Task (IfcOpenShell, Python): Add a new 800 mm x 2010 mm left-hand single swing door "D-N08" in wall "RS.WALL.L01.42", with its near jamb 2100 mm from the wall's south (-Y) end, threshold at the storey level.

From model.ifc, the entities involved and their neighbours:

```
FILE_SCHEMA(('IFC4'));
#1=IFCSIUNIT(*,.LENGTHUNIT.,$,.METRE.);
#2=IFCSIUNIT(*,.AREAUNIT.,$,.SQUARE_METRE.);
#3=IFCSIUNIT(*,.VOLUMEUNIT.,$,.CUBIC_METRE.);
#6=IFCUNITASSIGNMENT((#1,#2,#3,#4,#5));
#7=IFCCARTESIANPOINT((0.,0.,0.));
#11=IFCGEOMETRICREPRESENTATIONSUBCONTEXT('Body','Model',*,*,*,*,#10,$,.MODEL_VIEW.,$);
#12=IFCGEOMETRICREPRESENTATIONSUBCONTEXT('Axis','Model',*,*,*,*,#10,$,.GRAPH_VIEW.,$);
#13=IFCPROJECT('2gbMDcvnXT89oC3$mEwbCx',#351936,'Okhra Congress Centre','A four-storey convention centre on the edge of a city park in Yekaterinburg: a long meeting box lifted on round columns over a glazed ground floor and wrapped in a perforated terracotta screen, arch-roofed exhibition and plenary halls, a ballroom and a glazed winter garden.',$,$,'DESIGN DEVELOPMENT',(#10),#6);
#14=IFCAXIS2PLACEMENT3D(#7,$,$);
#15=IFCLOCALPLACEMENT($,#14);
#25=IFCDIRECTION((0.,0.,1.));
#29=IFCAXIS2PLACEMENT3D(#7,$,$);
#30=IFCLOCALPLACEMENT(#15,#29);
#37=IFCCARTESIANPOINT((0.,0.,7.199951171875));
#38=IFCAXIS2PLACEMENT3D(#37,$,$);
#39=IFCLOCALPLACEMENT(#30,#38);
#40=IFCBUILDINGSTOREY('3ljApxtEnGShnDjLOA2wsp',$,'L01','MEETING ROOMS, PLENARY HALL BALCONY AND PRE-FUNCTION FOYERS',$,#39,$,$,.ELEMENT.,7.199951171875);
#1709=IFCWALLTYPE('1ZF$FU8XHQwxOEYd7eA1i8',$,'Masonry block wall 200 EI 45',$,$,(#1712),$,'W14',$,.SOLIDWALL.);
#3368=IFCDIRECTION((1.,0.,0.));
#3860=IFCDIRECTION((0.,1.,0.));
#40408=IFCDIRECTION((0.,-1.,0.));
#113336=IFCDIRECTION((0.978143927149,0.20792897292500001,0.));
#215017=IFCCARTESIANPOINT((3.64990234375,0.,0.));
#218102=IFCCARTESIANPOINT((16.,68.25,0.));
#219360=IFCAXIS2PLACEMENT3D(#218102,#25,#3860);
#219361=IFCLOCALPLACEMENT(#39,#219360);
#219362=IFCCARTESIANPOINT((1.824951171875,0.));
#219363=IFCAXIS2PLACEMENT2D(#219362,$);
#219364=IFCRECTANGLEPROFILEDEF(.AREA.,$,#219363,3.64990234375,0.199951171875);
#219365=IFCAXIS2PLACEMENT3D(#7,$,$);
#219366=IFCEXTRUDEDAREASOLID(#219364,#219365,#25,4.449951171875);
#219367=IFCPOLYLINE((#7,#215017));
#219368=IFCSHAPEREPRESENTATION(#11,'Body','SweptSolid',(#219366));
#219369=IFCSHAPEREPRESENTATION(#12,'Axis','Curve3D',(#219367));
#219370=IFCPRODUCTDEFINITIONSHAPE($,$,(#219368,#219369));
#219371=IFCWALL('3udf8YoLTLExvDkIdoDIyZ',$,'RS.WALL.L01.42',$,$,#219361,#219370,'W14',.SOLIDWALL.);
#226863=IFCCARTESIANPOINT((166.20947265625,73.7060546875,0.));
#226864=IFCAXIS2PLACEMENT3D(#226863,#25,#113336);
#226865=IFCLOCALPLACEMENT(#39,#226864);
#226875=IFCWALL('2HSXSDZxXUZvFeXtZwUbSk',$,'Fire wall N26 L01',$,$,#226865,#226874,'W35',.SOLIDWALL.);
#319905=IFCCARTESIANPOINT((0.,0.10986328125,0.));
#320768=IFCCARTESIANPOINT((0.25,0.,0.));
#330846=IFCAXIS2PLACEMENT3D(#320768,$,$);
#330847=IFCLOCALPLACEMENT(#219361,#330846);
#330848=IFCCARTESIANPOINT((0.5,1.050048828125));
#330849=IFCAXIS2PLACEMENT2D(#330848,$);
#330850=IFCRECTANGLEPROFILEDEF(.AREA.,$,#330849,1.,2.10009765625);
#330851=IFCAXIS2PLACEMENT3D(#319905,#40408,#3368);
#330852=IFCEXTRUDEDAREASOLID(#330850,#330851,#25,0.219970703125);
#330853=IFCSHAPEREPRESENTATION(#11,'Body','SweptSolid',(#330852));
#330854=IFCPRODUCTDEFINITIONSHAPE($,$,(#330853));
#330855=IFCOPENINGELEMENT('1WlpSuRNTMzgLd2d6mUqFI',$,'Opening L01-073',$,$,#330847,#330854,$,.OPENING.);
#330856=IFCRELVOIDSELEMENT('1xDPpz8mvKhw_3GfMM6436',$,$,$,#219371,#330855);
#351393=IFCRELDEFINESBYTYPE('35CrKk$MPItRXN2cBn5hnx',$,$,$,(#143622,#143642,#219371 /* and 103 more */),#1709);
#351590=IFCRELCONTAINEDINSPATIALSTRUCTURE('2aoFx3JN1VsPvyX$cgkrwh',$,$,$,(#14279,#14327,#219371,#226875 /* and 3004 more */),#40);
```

```python
import numpy as np
import ifcopenshell
import ifcopenshell.api.feature
import ifcopenshell.api.geometry
import ifcopenshell.api.root
import ifcopenshell.api.spatial
import ifcopenshell.geom
import ifcopenshell.util.element
import ifcopenshell.util.placement
import ifcopenshell.util.representation
import ifcopenshell.util.shape
import ifcopenshell.util.unit

model = ifcopenshell.open("model.ifc")
unit_scale = ifcopenshell.util.unit.calculate_unit_scale(model)
settings = ifcopenshell.geom.settings()


def volume(element):
    """Net volume in cubic metres, openings subtracted."""
    shape = ifcopenshell.geom.create_shape(settings, element)
    return ifcopenshell.util.shape.get_volume(shape.geometry)


wall = model.by_guid("3udf8YoLTLExvDkIdoDIyZ")
storey = ifcopenshell.util.element.get_container(wall, ifc_class="IfcBuildingStorey")
context = ifcopenshell.util.representation.get_context(model, "Model", "Body", "MODEL_VIEW")
before = volume(wall)

width, height, from_end, sill = 0.8, 2.01, 2.1, 0.0  # metres

# The wall runs along its own X axis, and the end named is its -X end.
wall_shape = ifcopenshell.geom.create_shape(settings, wall)
x, y, z = ifcopenshell.util.shape.get_vertices(wall_shape.geometry).T
start = x.min() + from_end
face, thickness = float(y.min()), float(y.max() - y.min())
wall_matrix = ifcopenshell.util.placement.get_local_placement(wall.ObjectPlacement)
level = ifcopenshell.util.placement.get_local_placement(storey.ObjectPlacement)[2, 3]


def in_wall(x, y):
    """Placement at x, y metres in the wall's axes, at sill height."""
    matrix = wall_matrix.copy()
    matrix[:, 3] = wall_matrix @ np.array([x / unit_scale, y / unit_scale, 0.0, 1.0])
    matrix[2, 3] = level + sill / unit_scale
    return matrix


# Opening: a box that overshoots both wall faces by 50 mm.
opening = ifcopenshell.api.root.create_entity(model, ifc_class="IfcOpeningElement", predefined_type="OPENING")
box = ifcopenshell.api.geometry.add_wall_representation(
    model, context=context, length=width, height=height, thickness=thickness + 0.1
)
ifcopenshell.api.geometry.assign_representation(model, product=opening, representation=box)
ifcopenshell.api.geometry.edit_object_placement(model, product=opening, matrix=in_wall(start, face - 0.05), is_si=False)
ifcopenshell.api.feature.add_feature(model, feature=opening, element=wall)

door = ifcopenshell.api.root.create_entity(model, ifc_class="IfcDoor", name="D-N08", predefined_type="DOOR")
door.OverallWidth, door.OverallHeight = width / unit_scale, height / unit_scale
door.OperationType = "SINGLE_SWING_LEFT"
body = ifcopenshell.api.geometry.add_door_representation(
    model,
    context=context,
    overall_width=door.OverallWidth,
    overall_height=door.OverallHeight,
    operation_type="SINGLE_SWING_LEFT",
    lining_properties={"LiningDepth": thickness / unit_scale, "ThresholdDepth": thickness / unit_scale},
)
ifcopenshell.api.geometry.assign_representation(model, product=door, representation=body)
ifcopenshell.api.spatial.assign_container(model, products=[door], relating_structure=storey)
ifcopenshell.api.feature.add_filling(model, opening=opening, element=door)

# The lining spans the wall, so the door starts at the wall face.
ifcopenshell.api.geometry.edit_object_placement(model, product=door, matrix=in_wall(start, face), is_si=False)

after = volume(wall)

print(f"wall volume {before:.3f} -> {after:.3f} m3")

model.write("model_rev.ifc")
```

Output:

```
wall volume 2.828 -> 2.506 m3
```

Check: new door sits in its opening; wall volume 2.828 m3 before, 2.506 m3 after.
